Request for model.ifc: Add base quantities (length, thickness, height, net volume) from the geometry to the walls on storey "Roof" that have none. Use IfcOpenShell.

First a look at what the model holds.

```python
import ifcopenshell
import ifcopenshell.util.element
import ifcopenshell.util.unit

model = ifcopenshell.open("model.ifc")
print(model.schema)
for unit_type in ("LENGTHUNIT", "AREAUNIT", "VOLUMEUNIT"):
    print(unit_type, ifcopenshell.util.unit.calculate_unit_scale(model, unit_type))
storey = next(s for s in model.by_type("IfcBuildingStorey") if s.Name == "Roof")
walls = [e for e in ifcopenshell.util.element.get_decomposition(storey) if e.is_a("IfcWall")]
for e in sorted(walls, key=lambda e: e.id()):
    print(e.id(), e.is_a(), e.Name, list(ifcopenshell.util.element.get_psets(e, qtos_only=True)), sep=" | ")
```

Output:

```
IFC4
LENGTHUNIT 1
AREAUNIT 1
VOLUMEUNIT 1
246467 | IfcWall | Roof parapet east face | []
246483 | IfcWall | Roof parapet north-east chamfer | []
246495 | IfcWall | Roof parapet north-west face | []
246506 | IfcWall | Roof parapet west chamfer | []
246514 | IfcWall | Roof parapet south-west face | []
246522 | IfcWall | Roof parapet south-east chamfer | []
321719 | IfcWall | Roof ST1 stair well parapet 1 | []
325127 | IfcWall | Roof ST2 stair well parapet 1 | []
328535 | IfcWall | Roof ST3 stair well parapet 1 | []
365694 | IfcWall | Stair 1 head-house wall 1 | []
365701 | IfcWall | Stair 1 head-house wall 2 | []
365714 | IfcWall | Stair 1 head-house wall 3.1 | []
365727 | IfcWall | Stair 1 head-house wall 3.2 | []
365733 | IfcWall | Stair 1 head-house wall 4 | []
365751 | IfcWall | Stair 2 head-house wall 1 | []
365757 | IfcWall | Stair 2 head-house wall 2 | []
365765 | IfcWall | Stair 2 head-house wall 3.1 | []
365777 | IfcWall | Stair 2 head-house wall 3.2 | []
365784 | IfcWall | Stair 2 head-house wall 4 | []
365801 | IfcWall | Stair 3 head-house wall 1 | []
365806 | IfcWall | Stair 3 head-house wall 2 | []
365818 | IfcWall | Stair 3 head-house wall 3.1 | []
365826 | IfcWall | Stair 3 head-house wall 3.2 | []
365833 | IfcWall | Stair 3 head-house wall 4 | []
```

```python
import ifcopenshell
import ifcopenshell.api.pset
import ifcopenshell.geom
import ifcopenshell.util.element
import ifcopenshell.util.shape
import ifcopenshell.util.unit

model = ifcopenshell.open("model.ifc")
unit_scale = ifcopenshell.util.unit.calculate_unit_scale(model)
volume_scale = ifcopenshell.util.unit.calculate_unit_scale(model, "VOLUMEUNIT")
settings = ifcopenshell.geom.settings()

storey = next(s for s in model.by_type("IfcBuildingStorey") if s.Name == "Roof")
walls = [e for e in ifcopenshell.util.element.get_decomposition(storey) if e.is_a("IfcWall")]

for e in sorted(walls, key=lambda e: e.id()):
    if ifcopenshell.util.element.get_psets(e, qtos_only=True, should_inherit=False):
        continue
    # Geometry comes back in metres, in the element's own axes.
    shape = ifcopenshell.geom.create_shape(settings, e)
    values = {
        "Length": ifcopenshell.util.shape.get_x(shape.geometry) / unit_scale,
        "Width": ifcopenshell.util.shape.get_y(shape.geometry) / unit_scale,
        "Height": ifcopenshell.util.shape.get_z(shape.geometry) / unit_scale,
        "NetVolume": ifcopenshell.util.shape.get_volume(shape.geometry) / volume_scale,
    }
    qto = ifcopenshell.api.pset.add_qto(model, product=e, name="Qto_WallBaseQuantities")
    ifcopenshell.api.pset.edit_qto(model, qto=qto, properties=values)
    print(e.id(), {k: round(v, 3) for k, v in values.items()})

model.write("model_v2.ifc")
```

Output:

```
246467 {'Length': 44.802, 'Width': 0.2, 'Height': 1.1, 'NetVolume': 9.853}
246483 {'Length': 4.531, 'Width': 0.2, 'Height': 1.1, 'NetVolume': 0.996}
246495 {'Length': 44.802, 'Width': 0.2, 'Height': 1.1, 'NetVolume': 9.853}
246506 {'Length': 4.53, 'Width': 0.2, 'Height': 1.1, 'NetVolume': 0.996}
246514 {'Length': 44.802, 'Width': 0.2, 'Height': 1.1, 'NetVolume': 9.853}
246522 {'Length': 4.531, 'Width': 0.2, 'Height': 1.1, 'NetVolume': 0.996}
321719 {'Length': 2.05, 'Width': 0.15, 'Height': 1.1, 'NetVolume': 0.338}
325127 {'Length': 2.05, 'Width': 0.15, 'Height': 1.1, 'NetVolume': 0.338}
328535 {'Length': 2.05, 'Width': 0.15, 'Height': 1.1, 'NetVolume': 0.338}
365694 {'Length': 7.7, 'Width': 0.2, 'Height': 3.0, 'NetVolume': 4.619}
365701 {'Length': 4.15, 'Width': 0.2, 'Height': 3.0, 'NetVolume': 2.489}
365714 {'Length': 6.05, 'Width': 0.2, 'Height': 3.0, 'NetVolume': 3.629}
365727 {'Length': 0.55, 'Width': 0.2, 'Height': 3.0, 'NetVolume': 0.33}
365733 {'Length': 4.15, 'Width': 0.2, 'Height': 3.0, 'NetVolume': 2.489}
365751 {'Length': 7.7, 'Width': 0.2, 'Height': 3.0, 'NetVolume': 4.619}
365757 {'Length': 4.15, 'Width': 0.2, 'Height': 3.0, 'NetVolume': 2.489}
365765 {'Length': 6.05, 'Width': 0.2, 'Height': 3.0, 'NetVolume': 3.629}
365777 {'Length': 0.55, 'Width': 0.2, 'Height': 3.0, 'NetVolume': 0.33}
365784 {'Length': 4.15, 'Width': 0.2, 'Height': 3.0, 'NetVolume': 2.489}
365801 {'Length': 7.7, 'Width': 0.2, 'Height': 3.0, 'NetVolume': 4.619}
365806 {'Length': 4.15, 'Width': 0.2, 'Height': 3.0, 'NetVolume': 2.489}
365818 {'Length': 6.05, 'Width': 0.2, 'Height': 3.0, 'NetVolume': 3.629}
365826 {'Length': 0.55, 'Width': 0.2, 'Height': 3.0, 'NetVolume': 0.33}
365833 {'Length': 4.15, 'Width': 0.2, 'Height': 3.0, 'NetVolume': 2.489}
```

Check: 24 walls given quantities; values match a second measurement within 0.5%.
